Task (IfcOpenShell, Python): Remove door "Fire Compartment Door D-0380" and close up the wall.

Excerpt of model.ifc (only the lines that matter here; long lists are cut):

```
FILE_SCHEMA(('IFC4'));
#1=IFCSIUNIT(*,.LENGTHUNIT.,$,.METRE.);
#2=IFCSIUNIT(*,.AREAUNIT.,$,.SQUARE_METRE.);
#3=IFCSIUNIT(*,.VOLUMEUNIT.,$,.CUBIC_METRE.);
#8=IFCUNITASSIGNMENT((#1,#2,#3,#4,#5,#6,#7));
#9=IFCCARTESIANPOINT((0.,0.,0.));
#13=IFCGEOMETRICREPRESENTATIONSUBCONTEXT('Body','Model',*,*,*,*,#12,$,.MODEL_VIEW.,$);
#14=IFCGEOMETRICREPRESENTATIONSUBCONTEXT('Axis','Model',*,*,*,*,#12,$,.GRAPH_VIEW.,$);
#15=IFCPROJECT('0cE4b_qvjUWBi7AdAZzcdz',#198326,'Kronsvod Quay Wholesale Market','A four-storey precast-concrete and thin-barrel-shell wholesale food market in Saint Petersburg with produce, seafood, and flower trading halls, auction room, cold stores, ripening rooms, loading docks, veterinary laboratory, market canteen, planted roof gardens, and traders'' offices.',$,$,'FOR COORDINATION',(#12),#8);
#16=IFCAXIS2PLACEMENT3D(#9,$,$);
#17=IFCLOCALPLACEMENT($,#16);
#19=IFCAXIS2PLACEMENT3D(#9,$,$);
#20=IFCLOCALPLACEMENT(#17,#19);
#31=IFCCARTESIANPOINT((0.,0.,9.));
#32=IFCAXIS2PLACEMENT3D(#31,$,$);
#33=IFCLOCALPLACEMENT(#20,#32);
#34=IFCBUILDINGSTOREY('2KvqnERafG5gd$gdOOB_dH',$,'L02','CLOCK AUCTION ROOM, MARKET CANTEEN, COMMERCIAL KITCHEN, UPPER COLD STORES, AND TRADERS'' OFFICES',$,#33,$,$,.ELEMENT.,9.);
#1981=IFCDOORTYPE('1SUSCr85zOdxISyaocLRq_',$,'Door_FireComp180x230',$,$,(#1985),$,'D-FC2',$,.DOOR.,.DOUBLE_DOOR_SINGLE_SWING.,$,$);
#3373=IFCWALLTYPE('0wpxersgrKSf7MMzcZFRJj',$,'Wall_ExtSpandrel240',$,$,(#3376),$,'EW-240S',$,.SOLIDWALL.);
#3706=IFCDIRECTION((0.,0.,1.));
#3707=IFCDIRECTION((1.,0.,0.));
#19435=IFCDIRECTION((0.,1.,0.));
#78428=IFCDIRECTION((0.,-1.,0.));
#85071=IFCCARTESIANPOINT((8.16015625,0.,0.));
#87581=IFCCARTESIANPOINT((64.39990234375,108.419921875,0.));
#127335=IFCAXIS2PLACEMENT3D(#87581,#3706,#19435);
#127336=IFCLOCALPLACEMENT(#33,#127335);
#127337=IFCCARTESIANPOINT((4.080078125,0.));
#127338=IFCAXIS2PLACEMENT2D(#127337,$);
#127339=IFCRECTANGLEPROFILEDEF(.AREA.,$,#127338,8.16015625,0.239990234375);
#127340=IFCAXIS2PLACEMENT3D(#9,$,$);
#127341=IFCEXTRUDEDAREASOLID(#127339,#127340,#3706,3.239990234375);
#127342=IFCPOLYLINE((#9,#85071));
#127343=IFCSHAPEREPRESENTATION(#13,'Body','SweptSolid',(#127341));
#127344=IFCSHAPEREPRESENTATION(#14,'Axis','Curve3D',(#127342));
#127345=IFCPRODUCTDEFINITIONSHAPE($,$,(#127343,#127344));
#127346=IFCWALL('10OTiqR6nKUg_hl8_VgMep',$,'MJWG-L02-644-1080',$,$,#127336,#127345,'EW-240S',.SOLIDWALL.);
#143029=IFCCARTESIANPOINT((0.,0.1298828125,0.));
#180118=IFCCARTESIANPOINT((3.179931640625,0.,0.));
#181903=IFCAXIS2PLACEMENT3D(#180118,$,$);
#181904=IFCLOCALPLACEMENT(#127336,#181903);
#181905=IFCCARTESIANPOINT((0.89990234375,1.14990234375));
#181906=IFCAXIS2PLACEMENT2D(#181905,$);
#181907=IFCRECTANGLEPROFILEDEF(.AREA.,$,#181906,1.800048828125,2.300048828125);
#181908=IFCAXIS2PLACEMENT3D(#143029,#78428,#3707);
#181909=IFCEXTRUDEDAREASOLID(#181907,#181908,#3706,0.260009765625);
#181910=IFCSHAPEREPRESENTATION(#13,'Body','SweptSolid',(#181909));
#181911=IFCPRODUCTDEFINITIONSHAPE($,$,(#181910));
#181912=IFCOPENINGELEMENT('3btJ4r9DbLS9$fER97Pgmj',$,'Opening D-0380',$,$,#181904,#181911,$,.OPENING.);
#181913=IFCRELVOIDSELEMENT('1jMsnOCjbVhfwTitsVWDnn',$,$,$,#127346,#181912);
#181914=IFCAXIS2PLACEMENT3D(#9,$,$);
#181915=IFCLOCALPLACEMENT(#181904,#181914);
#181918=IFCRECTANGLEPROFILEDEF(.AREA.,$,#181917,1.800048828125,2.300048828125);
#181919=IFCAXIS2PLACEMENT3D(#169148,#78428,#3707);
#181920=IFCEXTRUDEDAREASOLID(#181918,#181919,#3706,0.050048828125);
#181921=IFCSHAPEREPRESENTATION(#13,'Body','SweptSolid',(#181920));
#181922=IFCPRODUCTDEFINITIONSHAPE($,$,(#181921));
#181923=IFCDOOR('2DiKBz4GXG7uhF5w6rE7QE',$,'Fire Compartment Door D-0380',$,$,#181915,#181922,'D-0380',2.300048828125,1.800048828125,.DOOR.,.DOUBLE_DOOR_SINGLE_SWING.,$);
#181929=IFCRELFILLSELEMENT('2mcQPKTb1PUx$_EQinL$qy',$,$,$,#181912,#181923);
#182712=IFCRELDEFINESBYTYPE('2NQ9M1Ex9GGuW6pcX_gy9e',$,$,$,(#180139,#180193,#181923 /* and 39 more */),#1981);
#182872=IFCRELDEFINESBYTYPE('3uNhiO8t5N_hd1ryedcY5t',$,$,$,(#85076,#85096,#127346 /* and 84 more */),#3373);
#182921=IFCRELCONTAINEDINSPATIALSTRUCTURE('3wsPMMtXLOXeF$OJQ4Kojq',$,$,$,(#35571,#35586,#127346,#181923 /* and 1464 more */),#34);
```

```python
import ifcopenshell
import ifcopenshell.api.feature
import ifcopenshell.api.root
import ifcopenshell.geom
import ifcopenshell.util.shape

model = ifcopenshell.open("model.ifc")
settings = ifcopenshell.geom.settings()


def volume(element):
    """Net volume in cubic metres, openings subtracted."""
    shape = ifcopenshell.geom.create_shape(settings, element)
    return ifcopenshell.util.shape.get_volume(shape.geometry)


door = model.by_guid("2DiKBz4GXG7uhF5w6rE7QE")
opening = door.FillsVoids[0].RelatingOpeningElement
wall = opening.VoidsElements[0].RelatingBuildingElement
before = volume(wall)

ifcopenshell.api.root.remove_product(model, product=door)
ifcopenshell.api.feature.remove_feature(model, feature=opening)

after = volume(wall)

print(f"wall volume {before:.3f} -> {after:.3f} m3")

model.write("model_updated.ifc")
```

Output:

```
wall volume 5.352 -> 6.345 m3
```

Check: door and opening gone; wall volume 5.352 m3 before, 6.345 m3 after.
